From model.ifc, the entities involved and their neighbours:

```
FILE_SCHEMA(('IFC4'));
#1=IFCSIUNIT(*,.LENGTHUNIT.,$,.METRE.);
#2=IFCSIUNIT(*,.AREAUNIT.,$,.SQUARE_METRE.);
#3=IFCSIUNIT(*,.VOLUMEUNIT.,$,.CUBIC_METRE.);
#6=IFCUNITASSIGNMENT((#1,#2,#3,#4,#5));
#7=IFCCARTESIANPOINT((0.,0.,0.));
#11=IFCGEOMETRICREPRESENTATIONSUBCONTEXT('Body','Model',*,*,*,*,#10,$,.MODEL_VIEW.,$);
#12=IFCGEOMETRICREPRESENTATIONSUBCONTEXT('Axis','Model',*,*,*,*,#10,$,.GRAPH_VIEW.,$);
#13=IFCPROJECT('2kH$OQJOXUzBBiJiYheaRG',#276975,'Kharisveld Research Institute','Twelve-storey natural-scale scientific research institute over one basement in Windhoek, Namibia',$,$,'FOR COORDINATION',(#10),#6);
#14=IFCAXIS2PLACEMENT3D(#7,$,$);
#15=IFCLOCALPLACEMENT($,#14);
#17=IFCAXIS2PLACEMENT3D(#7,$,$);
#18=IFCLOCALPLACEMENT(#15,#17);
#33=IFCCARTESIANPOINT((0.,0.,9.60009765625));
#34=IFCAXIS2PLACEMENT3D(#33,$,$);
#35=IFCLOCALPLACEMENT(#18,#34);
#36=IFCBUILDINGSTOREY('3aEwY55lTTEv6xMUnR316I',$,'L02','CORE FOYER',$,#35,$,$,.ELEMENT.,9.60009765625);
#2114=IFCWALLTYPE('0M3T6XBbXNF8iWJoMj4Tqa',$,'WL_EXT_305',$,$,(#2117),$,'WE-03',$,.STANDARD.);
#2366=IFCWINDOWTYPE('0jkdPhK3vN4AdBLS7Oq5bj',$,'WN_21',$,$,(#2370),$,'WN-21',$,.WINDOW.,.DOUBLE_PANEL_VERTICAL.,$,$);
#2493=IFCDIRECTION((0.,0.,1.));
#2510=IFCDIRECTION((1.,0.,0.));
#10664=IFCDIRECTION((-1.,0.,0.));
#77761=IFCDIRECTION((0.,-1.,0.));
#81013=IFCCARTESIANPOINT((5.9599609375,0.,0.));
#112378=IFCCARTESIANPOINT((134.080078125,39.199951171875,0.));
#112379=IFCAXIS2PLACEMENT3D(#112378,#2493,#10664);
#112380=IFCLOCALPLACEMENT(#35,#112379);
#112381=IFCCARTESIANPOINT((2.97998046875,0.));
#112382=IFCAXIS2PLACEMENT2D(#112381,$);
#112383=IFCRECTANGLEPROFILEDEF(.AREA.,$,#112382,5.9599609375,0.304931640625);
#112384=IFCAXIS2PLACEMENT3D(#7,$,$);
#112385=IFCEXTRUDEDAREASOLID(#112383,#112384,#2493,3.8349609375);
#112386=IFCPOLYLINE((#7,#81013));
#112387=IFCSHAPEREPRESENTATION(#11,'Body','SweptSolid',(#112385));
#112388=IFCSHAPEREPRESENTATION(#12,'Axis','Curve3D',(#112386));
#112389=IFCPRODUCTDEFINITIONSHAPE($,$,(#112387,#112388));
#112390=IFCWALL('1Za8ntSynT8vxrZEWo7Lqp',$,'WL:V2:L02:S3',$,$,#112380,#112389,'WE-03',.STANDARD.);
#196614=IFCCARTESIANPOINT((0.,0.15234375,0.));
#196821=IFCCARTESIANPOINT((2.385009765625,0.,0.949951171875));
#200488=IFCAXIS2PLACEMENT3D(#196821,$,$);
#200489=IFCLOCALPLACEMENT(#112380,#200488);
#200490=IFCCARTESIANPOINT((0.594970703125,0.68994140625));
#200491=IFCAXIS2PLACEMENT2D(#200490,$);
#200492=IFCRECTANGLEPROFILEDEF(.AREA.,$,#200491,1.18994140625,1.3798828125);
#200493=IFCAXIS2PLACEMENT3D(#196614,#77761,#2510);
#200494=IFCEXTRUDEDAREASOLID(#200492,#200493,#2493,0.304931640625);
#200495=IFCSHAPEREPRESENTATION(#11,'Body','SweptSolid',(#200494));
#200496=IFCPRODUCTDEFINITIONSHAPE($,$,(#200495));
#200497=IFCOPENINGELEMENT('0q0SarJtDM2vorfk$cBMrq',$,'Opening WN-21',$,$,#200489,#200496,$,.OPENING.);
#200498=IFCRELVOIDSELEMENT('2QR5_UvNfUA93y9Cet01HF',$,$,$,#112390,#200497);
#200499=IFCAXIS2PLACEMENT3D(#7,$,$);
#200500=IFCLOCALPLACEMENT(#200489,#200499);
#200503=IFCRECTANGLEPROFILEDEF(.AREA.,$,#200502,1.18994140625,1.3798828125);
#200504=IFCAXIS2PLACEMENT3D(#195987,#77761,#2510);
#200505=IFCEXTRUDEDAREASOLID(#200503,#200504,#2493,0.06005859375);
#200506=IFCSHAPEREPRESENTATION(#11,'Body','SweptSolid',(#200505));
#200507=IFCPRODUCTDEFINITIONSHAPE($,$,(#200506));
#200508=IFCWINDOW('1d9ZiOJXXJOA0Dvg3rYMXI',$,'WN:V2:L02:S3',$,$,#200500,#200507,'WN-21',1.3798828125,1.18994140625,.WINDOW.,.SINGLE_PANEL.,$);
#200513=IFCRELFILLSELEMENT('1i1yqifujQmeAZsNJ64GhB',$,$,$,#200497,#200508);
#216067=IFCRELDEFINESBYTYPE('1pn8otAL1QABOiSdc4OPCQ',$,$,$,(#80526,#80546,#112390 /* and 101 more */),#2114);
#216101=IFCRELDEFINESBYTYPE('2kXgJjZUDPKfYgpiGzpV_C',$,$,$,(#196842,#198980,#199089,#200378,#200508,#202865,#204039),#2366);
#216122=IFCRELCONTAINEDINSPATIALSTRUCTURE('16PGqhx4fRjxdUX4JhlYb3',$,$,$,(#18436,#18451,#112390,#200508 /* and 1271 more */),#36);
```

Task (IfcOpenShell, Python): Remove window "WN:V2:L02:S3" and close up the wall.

```python
import ifcopenshell
import ifcopenshell.api.feature
import ifcopenshell.api.root
import ifcopenshell.geom
import ifcopenshell.util.shape

model = ifcopenshell.open("model.ifc")
settings = ifcopenshell.geom.settings()


def volume(element):
    """Net volume in cubic metres, openings subtracted."""
    shape = ifcopenshell.geom.create_shape(settings, element)
    return ifcopenshell.util.shape.get_volume(shape.geometry)


window = model.by_guid("1d9ZiOJXXJOA0Dvg3rYMXI")
opening = window.FillsVoids[0].RelatingOpeningElement
wall = opening.VoidsElements[0].RelatingBuildingElement
before = volume(wall)

ifcopenshell.api.root.remove_product(model, product=window)
ifcopenshell.api.feature.remove_feature(model, feature=opening)

after = volume(wall)

print(f"wall volume {before:.3f} -> {after:.3f} m3")

model.write("model-out.ifc")
```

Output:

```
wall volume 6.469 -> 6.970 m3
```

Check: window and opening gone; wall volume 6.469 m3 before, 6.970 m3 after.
